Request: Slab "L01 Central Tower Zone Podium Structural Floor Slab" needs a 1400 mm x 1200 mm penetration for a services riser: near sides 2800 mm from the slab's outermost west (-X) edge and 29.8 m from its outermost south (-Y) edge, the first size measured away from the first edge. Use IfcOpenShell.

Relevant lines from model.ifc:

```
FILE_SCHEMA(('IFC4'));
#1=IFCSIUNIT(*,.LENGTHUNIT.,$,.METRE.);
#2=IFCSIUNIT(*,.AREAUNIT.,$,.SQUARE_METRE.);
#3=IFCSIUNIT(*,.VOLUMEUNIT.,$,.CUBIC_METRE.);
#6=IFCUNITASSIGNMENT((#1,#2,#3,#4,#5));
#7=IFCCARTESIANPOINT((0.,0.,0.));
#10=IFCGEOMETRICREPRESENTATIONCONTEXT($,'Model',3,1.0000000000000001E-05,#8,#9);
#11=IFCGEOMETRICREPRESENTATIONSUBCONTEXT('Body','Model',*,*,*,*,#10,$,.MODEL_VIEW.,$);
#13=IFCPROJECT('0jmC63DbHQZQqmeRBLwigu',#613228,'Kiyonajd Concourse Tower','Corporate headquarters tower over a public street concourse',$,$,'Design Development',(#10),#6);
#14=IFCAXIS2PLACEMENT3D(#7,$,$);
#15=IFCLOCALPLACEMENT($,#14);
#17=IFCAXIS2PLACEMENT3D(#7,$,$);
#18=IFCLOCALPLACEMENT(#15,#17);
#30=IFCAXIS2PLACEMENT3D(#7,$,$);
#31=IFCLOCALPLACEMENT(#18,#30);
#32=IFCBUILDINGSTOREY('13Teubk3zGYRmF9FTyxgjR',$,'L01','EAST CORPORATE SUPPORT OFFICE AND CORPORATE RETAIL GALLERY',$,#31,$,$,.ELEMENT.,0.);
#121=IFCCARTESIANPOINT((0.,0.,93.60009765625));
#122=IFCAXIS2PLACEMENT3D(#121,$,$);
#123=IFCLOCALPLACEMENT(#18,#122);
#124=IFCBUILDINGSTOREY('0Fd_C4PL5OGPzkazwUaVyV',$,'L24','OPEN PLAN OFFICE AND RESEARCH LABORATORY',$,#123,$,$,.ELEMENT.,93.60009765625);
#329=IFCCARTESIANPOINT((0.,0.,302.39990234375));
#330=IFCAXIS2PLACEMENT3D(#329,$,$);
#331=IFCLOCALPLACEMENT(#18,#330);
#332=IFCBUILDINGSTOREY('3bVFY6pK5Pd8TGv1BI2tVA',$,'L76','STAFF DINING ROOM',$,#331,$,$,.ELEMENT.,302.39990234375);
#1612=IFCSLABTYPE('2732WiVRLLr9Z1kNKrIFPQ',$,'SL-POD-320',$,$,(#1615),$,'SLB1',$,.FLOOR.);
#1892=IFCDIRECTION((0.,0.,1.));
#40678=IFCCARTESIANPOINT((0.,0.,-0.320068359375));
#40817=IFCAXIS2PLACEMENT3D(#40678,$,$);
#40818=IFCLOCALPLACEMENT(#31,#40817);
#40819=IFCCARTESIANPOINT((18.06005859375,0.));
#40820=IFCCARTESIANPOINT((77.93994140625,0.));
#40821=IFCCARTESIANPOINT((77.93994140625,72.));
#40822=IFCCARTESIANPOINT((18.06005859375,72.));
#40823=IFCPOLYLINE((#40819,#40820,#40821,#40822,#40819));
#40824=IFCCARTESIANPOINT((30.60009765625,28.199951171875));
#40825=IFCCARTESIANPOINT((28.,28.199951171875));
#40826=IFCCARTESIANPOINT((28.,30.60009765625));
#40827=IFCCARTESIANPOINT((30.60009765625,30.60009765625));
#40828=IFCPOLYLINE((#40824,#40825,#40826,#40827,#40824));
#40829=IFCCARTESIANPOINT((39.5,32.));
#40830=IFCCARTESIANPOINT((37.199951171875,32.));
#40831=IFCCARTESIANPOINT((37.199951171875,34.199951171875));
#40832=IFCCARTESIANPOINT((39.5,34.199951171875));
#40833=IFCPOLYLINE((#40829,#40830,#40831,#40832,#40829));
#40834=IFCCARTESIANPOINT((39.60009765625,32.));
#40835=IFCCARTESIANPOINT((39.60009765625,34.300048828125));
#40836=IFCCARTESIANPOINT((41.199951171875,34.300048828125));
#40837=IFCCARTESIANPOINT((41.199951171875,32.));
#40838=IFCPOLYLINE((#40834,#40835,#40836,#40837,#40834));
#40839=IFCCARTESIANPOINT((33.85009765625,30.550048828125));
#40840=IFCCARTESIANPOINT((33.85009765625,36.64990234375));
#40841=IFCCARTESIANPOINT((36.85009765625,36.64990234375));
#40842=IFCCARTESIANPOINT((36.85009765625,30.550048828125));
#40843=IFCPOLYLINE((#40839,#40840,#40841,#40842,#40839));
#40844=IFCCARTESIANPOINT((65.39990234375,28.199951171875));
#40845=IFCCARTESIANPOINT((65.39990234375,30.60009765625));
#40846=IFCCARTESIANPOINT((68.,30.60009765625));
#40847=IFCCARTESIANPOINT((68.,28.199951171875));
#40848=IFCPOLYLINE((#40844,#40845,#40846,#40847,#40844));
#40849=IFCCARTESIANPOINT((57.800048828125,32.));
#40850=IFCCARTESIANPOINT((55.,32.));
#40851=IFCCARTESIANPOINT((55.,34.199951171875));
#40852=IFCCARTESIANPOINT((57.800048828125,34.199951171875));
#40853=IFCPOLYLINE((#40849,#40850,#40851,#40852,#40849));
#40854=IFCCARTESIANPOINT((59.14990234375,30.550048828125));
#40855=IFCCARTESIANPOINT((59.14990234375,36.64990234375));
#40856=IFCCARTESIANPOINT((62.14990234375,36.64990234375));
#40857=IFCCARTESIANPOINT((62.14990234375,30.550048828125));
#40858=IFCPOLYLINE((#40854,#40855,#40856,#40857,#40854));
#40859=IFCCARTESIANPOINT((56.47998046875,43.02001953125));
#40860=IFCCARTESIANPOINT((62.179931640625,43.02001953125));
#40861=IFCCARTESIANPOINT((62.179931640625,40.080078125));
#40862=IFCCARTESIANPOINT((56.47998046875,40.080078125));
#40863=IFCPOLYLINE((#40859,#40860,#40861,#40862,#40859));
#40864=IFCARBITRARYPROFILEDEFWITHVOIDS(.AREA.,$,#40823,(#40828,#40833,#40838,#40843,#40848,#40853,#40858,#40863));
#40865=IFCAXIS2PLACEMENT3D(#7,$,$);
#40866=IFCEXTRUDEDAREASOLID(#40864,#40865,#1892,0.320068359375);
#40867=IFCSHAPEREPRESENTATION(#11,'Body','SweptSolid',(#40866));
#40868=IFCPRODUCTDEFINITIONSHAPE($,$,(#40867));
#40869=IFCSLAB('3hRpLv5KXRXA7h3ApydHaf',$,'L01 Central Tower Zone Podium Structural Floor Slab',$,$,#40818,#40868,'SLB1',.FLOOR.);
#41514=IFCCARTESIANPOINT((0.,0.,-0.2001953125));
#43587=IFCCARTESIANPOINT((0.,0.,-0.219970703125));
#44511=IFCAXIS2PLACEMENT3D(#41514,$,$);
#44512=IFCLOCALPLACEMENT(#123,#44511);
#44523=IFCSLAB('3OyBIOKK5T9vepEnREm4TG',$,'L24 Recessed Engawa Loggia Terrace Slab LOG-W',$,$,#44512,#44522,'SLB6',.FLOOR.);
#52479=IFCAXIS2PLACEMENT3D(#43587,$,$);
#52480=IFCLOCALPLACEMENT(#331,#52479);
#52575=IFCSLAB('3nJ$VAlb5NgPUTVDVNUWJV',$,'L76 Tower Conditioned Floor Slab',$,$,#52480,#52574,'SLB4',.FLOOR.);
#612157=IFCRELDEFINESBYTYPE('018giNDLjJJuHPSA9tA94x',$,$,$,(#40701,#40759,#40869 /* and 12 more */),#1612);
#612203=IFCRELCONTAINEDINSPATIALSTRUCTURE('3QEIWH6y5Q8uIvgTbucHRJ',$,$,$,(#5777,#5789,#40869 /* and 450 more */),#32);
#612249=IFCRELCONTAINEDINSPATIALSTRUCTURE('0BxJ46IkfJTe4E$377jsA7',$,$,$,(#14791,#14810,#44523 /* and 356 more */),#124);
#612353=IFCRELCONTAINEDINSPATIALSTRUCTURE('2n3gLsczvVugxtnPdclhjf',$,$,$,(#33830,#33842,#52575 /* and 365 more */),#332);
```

```python
import numpy as np
import ifcopenshell
import ifcopenshell.api.feature
import ifcopenshell.api.geometry
import ifcopenshell.api.root
import ifcopenshell.geom
import ifcopenshell.util.placement
import ifcopenshell.util.representation
import ifcopenshell.util.shape
import ifcopenshell.util.unit

model = ifcopenshell.open("model.ifc")
unit_scale = ifcopenshell.util.unit.calculate_unit_scale(model)
settings = ifcopenshell.geom.settings()


def volume(element):
    """Net volume in cubic metres, openings subtracted."""
    shape = ifcopenshell.geom.create_shape(settings, element)
    return ifcopenshell.util.shape.get_volume(shape.geometry)


slab = model.by_id(40869)
before = volume(slab)

# Extent in the slab's own axes, in metres. The edges named are its -X and -Y sides.
slab_shape = ifcopenshell.geom.create_shape(settings, slab)
vertices = ifcopenshell.util.shape.get_vertices(slab_shape.geometry)
x_min, y_min, bottom = vertices.min(axis=0)
top = vertices[:, 2].max()

opening = ifcopenshell.api.root.create_entity(model, ifc_class="IfcOpeningElement", name="Services riser opening", predefined_type="OPENING")
context = ifcopenshell.util.representation.get_context(model, "Model", "Body", "MODEL_VIEW")
width, depth = 1.4, 1.2
outline = [(0.0, 0.0), (width, 0.0), (width, depth), (0.0, depth), (0.0, 0.0)]
# Overshoot both faces by 50 mm so the cut is clean.
shape = ifcopenshell.api.geometry.add_slab_representation(
    model, context=context, depth=top - bottom + 0.1, polyline=outline
)
ifcopenshell.api.geometry.assign_representation(model, product=opening, representation=shape)

matrix = ifcopenshell.util.placement.get_local_placement(slab.ObjectPlacement)
matrix[:, 3] = matrix @ np.append(np.array([x_min + 2.8, y_min + 29.8, bottom - 0.05]) / unit_scale, 1.0)
ifcopenshell.api.geometry.edit_object_placement(model, product=opening, matrix=matrix, is_si=False)
ifcopenshell.api.feature.add_feature(model, feature=opening, element=slab)

after = volume(slab)

print(f"slab volume {before:.3f} -> {after:.3f} m3")

model.write("model_rev.ifc")
```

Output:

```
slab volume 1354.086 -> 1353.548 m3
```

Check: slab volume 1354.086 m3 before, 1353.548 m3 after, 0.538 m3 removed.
